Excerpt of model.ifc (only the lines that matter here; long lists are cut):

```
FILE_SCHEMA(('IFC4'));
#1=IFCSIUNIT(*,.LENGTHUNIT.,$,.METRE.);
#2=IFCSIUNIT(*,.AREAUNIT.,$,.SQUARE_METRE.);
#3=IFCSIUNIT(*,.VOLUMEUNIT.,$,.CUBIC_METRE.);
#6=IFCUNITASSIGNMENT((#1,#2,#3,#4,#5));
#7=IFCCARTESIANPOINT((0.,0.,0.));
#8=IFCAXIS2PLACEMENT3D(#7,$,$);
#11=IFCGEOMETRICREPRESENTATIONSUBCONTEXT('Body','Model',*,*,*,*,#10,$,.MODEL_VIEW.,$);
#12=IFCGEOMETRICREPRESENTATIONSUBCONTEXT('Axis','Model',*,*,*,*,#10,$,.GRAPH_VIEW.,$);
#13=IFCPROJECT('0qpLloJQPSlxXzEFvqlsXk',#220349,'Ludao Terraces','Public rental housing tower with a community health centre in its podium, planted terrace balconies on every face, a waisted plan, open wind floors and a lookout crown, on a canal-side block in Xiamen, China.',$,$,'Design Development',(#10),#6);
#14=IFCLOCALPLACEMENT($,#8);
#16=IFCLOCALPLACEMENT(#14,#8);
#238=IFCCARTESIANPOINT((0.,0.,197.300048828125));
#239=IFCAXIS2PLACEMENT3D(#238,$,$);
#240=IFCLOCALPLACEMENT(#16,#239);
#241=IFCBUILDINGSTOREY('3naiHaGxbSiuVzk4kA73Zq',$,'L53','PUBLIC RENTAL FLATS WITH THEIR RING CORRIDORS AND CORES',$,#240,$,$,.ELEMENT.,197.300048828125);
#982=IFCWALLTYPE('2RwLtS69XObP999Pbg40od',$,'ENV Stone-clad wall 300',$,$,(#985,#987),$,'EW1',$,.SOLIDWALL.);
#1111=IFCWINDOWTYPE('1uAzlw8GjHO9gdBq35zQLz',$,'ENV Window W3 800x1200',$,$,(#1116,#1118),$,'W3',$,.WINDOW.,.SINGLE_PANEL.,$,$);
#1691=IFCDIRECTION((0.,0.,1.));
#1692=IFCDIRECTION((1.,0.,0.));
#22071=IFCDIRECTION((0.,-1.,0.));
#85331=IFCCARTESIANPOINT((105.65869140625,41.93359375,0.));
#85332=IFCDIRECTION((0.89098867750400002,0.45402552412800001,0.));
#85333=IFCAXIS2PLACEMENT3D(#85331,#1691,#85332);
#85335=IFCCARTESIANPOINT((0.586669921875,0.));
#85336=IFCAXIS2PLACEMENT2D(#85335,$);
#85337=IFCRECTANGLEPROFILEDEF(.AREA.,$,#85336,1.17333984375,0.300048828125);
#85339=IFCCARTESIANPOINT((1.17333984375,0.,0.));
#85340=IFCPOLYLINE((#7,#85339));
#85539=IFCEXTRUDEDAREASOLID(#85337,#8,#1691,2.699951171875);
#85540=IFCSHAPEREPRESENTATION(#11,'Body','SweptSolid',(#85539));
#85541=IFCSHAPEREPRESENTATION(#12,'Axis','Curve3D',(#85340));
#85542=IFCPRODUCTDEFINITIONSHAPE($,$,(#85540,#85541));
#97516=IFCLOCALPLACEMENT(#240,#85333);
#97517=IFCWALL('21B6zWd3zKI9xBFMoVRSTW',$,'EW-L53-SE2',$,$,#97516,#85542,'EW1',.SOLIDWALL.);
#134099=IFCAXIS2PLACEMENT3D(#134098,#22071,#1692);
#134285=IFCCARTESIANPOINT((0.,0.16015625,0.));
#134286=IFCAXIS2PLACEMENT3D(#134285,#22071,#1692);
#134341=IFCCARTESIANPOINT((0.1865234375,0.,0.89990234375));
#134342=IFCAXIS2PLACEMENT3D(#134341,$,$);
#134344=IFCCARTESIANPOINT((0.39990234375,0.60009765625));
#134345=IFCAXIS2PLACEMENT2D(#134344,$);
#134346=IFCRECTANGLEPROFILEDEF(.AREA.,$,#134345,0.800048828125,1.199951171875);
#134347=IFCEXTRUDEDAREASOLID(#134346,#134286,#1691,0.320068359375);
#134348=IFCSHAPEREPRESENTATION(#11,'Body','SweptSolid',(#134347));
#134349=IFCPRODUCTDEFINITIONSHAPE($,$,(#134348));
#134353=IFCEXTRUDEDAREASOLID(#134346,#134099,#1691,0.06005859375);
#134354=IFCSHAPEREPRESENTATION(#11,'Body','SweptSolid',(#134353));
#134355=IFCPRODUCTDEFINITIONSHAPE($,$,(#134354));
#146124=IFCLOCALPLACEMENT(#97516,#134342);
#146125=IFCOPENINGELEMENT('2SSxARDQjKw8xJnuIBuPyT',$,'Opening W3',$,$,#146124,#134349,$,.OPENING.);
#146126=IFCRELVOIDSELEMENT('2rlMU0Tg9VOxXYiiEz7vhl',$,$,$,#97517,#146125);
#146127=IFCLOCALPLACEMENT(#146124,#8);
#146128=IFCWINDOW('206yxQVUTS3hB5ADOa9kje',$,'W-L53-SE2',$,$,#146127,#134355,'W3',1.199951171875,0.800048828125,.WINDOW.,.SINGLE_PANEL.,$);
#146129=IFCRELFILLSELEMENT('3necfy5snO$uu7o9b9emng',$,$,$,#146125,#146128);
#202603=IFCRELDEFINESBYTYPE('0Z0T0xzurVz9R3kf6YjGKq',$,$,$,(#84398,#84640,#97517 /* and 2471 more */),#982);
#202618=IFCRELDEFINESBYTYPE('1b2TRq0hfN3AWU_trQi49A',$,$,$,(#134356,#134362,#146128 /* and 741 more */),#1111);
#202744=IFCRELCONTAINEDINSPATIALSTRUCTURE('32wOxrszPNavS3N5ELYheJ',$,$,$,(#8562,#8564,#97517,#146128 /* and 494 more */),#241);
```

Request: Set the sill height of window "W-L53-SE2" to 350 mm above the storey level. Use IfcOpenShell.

```python
import numpy as np
import ifcopenshell
import ifcopenshell.api.geometry
import ifcopenshell.geom
import ifcopenshell.util.element
import ifcopenshell.util.placement
import ifcopenshell.util.shape
import ifcopenshell.util.unit

model = ifcopenshell.open("model.ifc")
unit_scale = ifcopenshell.util.unit.calculate_unit_scale(model)

window = model.by_guid("206yxQVUTS3hB5ADOa9kje")
opening = window.FillsVoids[0].RelatingOpeningElement
storey = ifcopenshell.util.element.get_container(window, ifc_class="IfcBuildingStorey")
level = ifcopenshell.util.placement.get_local_placement(storey.ObjectPlacement)[2, 3]

# The opening's origin need not be at the sill, so measure its lowest point.
shape = ifcopenshell.geom.create_shape(ifcopenshell.geom.settings(), opening)
bottom = ifcopenshell.util.shape.get_shape_bottom_elevation(shape, shape.geometry) / unit_scale
dz = level + 0.35 / unit_scale - bottom

shift = np.array([0.0, 0.0, dz])
# The window is placed relative to its opening, so it follows when the opening moves.
matrix = ifcopenshell.util.placement.get_local_placement(opening.ObjectPlacement)
matrix[:3, 3] += shift
ifcopenshell.api.geometry.edit_object_placement(
    model, product=opening, matrix=matrix, is_si=False, should_transform_children=True
)

print(f"moved by {dz * unit_scale:+.3f} m")

model.write("model_rev.ifc")
```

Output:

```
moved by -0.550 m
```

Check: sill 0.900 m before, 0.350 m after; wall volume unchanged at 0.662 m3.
